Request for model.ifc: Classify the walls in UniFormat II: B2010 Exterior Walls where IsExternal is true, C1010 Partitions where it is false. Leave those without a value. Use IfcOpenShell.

First a look at what the model holds.

```python
import ifcopenshell
import ifcopenshell.util.element

model = ifcopenshell.open("model.ifc")
print(model.schema)
print("classifications:", [c.Name for c in model.by_type("IfcClassification")])
values = [ifcopenshell.util.element.get_pset(e, "Pset_WallCommon", "IsExternal") for e in model.by_type("IfcWall")]
for value in (True, False, None):
    print("IsExternal", value, values.count(value))
```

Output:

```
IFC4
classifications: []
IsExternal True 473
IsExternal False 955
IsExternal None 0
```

```python
import ifcopenshell
import ifcopenshell.api.classification
import ifcopenshell.util.element

model = ifcopenshell.open("model.ifc")

system = ifcopenshell.api.classification.add_classification(model, classification="UniFormat II")

walls = model.by_type("IfcWall")
external = {e: ifcopenshell.util.element.get_pset(e, "Pset_WallCommon", "IsExternal") for e in walls}
for flag, code, name in ((True, "B2010", "Exterior Walls"), (False, "C1010", "Partitions")):
    products = [e for e in walls if external[e] is flag]
    ifcopenshell.api.classification.add_reference(
        model, products=products, classification=system, identification=code, name=name
    )
    print(code, len(products))

model.write("model-out.ifc")
```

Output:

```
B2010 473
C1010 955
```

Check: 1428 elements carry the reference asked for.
